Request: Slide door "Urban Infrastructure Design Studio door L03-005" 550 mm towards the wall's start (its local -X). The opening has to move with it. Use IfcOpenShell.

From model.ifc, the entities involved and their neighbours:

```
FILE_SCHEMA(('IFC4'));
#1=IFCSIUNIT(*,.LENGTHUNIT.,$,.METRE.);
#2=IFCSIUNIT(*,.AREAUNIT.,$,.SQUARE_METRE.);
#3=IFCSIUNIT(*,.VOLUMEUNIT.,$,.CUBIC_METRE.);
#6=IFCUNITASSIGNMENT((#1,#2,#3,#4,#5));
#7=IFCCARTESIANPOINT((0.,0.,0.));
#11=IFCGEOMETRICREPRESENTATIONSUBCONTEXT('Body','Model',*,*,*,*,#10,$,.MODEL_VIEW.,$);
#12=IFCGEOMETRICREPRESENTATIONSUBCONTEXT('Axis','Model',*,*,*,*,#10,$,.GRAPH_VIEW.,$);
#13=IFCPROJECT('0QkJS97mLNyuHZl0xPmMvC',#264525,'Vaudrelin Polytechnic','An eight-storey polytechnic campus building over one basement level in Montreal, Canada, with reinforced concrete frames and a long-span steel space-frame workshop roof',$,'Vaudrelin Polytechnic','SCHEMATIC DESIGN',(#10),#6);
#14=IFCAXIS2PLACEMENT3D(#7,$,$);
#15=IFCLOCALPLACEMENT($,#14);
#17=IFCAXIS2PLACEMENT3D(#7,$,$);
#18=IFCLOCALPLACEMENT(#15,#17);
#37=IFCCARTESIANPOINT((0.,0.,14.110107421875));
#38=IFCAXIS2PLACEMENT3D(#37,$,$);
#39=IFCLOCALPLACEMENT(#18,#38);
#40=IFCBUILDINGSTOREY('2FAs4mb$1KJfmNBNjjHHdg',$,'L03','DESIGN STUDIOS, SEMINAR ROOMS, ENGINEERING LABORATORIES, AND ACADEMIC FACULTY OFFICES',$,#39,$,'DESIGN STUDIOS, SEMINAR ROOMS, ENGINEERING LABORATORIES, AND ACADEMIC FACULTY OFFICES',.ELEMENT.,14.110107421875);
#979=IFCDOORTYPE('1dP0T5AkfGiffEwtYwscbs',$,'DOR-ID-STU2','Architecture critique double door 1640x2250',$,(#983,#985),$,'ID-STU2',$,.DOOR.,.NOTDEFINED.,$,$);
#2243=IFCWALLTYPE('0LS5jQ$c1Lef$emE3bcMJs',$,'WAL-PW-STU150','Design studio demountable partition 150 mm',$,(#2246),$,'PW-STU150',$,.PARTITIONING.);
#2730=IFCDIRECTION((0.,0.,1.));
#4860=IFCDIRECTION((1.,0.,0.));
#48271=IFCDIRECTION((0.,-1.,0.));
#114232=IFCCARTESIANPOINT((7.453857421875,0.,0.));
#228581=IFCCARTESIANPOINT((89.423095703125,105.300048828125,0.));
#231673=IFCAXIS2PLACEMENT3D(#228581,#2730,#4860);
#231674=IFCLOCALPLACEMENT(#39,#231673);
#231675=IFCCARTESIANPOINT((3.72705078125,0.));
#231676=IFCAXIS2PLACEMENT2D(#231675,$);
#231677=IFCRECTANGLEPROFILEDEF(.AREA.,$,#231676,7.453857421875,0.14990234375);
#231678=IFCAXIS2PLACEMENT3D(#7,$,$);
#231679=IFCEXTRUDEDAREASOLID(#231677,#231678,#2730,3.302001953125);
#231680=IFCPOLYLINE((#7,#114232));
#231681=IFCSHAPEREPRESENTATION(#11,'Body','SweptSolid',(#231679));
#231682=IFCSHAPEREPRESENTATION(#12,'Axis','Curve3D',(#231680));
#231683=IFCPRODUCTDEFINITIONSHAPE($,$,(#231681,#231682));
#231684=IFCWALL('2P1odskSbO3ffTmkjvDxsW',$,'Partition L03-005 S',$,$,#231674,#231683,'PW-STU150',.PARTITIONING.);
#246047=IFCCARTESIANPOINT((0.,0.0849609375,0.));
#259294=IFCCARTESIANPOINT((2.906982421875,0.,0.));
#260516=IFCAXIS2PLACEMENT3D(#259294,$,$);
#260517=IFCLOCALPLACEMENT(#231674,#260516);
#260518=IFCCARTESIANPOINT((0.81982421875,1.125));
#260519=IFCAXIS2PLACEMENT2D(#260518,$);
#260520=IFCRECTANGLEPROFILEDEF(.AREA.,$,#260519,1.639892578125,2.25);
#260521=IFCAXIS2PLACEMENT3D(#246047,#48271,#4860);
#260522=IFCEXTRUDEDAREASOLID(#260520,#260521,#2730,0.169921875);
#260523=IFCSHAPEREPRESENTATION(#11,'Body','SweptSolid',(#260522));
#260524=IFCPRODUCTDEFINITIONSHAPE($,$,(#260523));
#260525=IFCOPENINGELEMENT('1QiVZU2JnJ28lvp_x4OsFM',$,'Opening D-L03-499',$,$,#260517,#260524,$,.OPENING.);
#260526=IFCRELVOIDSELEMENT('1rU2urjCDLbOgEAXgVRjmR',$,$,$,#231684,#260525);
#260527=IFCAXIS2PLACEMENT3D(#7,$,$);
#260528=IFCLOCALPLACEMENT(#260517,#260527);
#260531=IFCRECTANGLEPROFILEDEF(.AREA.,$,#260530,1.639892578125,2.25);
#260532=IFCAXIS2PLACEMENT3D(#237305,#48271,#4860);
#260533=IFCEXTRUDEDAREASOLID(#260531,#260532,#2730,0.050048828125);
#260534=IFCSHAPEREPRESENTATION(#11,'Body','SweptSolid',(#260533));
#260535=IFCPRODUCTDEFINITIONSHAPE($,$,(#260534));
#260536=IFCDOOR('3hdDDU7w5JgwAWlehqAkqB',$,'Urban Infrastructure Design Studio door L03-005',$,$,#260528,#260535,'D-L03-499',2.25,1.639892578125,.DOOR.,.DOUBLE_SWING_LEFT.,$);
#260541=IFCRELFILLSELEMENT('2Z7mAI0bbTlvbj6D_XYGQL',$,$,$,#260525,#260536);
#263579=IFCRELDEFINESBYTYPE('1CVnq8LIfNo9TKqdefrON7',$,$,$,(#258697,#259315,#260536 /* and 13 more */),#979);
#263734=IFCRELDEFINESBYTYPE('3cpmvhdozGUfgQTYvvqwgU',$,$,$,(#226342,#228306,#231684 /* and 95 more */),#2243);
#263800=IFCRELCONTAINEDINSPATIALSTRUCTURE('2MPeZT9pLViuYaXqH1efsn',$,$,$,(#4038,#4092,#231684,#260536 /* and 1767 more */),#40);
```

```python
import ifcopenshell
import ifcopenshell.api.geometry
import ifcopenshell.util.placement

model = ifcopenshell.open("model.ifc")

door = model.by_guid("3hdDDU7w5JgwAWlehqAkqB")
opening = door.FillsVoids[0].RelatingOpeningElement
wall = opening.VoidsElements[0].RelatingBuildingElement

wall_matrix = ifcopenshell.util.placement.get_local_placement(wall.ObjectPlacement)
shift = wall_matrix[:3, 0] * -0.55
before = ifcopenshell.util.placement.get_local_placement(door.ObjectPlacement)[:3, 3].copy()

# The door is placed relative to its opening, so it follows when the opening moves.
matrix = ifcopenshell.util.placement.get_local_placement(opening.ObjectPlacement)
matrix[:3, 3] += shift
ifcopenshell.api.geometry.edit_object_placement(
    model, product=opening, matrix=matrix, is_si=False, should_transform_children=True
)

after = ifcopenshell.util.placement.get_local_placement(door.ObjectPlacement)[:3, 3]
print("door moved by", (after - before).round(3) + 0.0)

model.write("model_updated.ifc")
```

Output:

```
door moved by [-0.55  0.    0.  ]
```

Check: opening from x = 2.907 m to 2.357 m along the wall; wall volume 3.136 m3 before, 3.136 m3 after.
